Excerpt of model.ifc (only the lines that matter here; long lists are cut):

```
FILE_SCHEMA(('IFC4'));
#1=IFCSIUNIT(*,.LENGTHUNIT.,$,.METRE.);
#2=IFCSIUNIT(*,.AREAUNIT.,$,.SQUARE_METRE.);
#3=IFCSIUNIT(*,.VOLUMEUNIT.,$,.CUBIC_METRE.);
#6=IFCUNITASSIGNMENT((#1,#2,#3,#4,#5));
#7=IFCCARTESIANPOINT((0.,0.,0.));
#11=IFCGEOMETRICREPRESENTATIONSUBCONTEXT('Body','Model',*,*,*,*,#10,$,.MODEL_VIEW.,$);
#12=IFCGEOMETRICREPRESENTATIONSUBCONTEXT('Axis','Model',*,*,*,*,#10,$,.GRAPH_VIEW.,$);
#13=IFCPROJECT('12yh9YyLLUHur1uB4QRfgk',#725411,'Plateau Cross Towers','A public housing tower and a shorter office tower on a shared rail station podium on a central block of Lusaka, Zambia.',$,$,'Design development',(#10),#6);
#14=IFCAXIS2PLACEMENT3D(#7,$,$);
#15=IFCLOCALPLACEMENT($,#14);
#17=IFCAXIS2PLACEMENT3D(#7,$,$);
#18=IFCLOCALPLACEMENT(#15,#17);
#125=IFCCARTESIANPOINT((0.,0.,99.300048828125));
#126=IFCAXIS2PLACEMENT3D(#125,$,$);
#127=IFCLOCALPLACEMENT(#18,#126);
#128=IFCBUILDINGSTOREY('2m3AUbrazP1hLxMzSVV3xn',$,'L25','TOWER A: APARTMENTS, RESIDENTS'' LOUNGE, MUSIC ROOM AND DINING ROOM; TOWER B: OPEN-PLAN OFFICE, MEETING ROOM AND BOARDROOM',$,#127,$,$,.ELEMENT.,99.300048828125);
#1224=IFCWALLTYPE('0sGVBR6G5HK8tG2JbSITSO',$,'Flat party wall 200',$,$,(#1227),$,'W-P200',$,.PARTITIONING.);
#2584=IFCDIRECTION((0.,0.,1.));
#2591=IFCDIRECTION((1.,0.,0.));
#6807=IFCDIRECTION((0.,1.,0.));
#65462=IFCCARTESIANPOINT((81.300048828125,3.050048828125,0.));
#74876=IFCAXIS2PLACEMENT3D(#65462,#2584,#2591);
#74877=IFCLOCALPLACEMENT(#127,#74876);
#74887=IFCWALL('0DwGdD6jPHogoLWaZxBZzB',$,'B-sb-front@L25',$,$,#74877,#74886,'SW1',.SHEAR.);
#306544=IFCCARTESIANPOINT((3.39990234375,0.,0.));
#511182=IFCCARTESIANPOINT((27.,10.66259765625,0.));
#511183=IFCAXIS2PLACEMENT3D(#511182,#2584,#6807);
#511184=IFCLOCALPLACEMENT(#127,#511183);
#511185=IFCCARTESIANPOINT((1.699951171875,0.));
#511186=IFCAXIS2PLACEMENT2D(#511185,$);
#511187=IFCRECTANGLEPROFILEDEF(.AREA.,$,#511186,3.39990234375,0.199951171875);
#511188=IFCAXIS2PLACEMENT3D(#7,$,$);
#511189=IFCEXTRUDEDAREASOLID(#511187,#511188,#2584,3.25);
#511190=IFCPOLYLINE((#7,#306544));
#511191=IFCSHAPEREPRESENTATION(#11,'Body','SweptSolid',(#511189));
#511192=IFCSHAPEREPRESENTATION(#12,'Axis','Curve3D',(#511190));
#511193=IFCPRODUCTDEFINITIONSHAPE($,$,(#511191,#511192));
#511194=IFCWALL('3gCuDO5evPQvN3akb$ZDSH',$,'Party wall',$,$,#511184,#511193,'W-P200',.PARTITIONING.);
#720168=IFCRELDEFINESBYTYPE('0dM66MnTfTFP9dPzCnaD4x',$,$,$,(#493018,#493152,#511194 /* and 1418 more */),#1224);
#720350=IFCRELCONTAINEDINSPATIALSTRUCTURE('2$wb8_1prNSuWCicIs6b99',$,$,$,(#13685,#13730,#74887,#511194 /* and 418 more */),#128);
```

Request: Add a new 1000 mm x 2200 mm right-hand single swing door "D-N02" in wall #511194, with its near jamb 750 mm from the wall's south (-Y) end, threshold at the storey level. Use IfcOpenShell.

```python
import numpy as np
import ifcopenshell
import ifcopenshell.api.feature
import ifcopenshell.api.geometry
import ifcopenshell.api.root
import ifcopenshell.api.spatial
import ifcopenshell.geom
import ifcopenshell.util.element
import ifcopenshell.util.placement
import ifcopenshell.util.representation
import ifcopenshell.util.shape
import ifcopenshell.util.unit

model = ifcopenshell.open("model.ifc")
unit_scale = ifcopenshell.util.unit.calculate_unit_scale(model)
settings = ifcopenshell.geom.settings()


def volume(element):
    """Net volume in cubic metres, openings subtracted."""
    shape = ifcopenshell.geom.create_shape(settings, element)
    return ifcopenshell.util.shape.get_volume(shape.geometry)


wall = model.by_guid("3gCuDO5evPQvN3akb$ZDSH")
storey = ifcopenshell.util.element.get_container(wall, ifc_class="IfcBuildingStorey")
context = ifcopenshell.util.representation.get_context(model, "Model", "Body", "MODEL_VIEW")
before = volume(wall)

width, height, from_end, sill = 1, 2.2, 0.75, 0.0  # metres

# The wall runs along its own X axis, and the end named is its -X end.
wall_shape = ifcopenshell.geom.create_shape(settings, wall)
x, y, z = ifcopenshell.util.shape.get_vertices(wall_shape.geometry).T
start = x.min() + from_end
face, thickness = float(y.min()), float(y.max() - y.min())
wall_matrix = ifcopenshell.util.placement.get_local_placement(wall.ObjectPlacement)
level = ifcopenshell.util.placement.get_local_placement(storey.ObjectPlacement)[2, 3]


def in_wall(x, y):
    """Placement at x, y metres in the wall's axes, at sill height."""
    matrix = wall_matrix.copy()
    matrix[:, 3] = wall_matrix @ np.array([x / unit_scale, y / unit_scale, 0.0, 1.0])
    matrix[2, 3] = level + sill / unit_scale
    return matrix


# Opening: a box that overshoots both wall faces by 50 mm.
opening = ifcopenshell.api.root.create_entity(model, ifc_class="IfcOpeningElement", predefined_type="OPENING")
box = ifcopenshell.api.geometry.add_wall_representation(
    model, context=context, length=width, height=height, thickness=thickness + 0.1
)
ifcopenshell.api.geometry.assign_representation(model, product=opening, representation=box)
ifcopenshell.api.geometry.edit_object_placement(model, product=opening, matrix=in_wall(start, face - 0.05), is_si=False)
ifcopenshell.api.feature.add_feature(model, feature=opening, element=wall)

door = ifcopenshell.api.root.create_entity(model, ifc_class="IfcDoor", name="D-N02", predefined_type="DOOR")
door.OverallWidth, door.OverallHeight = width / unit_scale, height / unit_scale
door.OperationType = "SINGLE_SWING_RIGHT"
body = ifcopenshell.api.geometry.add_door_representation(
    model,
    context=context,
    overall_width=door.OverallWidth,
    overall_height=door.OverallHeight,
    operation_type="SINGLE_SWING_RIGHT",
    lining_properties={"LiningDepth": thickness / unit_scale, "ThresholdDepth": thickness / unit_scale},
)
ifcopenshell.api.geometry.assign_representation(model, product=door, representation=body)
ifcopenshell.api.spatial.assign_container(model, products=[door], relating_structure=storey)
ifcopenshell.api.feature.add_filling(model, opening=opening, element=door)

# The lining spans the wall, so the door starts at the wall face.
ifcopenshell.api.geometry.edit_object_placement(model, product=door, matrix=in_wall(start, face), is_si=False)

after = volume(wall)

print(f"wall volume {before:.3f} -> {after:.3f} m3")

model.write("model_rev.ifc")
```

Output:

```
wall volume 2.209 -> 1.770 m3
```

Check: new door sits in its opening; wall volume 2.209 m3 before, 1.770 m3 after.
